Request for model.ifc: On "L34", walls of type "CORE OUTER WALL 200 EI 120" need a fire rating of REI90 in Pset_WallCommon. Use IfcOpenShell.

First a look at what the model holds.

```python
import ifcopenshell
import ifcopenshell.util.element

model = ifcopenshell.open("model.ifc")
print(model.schema)
storey = next(s for s in model.by_type("IfcBuildingStorey") if s.Name == "L34")
walls = [e for e in ifcopenshell.util.element.get_decomposition(storey) if e.is_a("IfcWall")]
seen = {}
for e in walls:
    element_type = ifcopenshell.util.element.get_type(e)
    key = (element_type.Name if element_type != e and element_type else None, ifcopenshell.util.element.get_pset(e, "Pset_WallCommon", "FireRating"))
    seen[key] = seen.get(key, 0) + 1
for (name, value), count in sorted(seen.items(), key=str):
    print(count, "x", name, "|", value)
```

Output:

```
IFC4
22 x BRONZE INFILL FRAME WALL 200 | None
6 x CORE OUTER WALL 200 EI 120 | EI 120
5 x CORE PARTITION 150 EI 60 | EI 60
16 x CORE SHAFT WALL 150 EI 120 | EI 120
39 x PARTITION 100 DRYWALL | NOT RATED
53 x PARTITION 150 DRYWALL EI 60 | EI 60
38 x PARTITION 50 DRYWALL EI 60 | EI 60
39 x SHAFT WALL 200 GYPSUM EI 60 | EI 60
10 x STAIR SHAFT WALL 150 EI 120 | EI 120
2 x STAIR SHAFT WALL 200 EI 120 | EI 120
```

```python
import ifcopenshell
import ifcopenshell.api.pset
import ifcopenshell.util.element

model = ifcopenshell.open("model.ifc")

storey = next(s for s in model.by_type("IfcBuildingStorey") if s.Name == "L34")
walls = [e for e in ifcopenshell.util.element.get_decomposition(storey) if e.is_a("IfcWall")]

count = 0
for e in walls:
    element_type = ifcopenshell.util.element.get_type(e)
    if element_type in (None, e) or element_type.Name != "CORE OUTER WALL 200 EI 120":
        continue
    found = ifcopenshell.util.element.get_pset(e, "Pset_WallCommon", should_inherit=False)
    if found:
        pset = model.by_id(found["id"])
        if len(ifcopenshell.util.element.get_elements_by_pset(pset)) > 1:
            pset = ifcopenshell.api.pset.unshare_pset(model, products=[e], pset=pset)[0]
    else:
        pset = ifcopenshell.api.pset.add_pset(model, product=e, name="Pset_WallCommon")
    ifcopenshell.api.pset.edit_pset(model, pset=pset, properties={"FireRating": "REI90"})
    count += 1

print(count, "walls updated")

model.write("model_v2.ifc")
```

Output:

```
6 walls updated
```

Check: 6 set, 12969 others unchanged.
